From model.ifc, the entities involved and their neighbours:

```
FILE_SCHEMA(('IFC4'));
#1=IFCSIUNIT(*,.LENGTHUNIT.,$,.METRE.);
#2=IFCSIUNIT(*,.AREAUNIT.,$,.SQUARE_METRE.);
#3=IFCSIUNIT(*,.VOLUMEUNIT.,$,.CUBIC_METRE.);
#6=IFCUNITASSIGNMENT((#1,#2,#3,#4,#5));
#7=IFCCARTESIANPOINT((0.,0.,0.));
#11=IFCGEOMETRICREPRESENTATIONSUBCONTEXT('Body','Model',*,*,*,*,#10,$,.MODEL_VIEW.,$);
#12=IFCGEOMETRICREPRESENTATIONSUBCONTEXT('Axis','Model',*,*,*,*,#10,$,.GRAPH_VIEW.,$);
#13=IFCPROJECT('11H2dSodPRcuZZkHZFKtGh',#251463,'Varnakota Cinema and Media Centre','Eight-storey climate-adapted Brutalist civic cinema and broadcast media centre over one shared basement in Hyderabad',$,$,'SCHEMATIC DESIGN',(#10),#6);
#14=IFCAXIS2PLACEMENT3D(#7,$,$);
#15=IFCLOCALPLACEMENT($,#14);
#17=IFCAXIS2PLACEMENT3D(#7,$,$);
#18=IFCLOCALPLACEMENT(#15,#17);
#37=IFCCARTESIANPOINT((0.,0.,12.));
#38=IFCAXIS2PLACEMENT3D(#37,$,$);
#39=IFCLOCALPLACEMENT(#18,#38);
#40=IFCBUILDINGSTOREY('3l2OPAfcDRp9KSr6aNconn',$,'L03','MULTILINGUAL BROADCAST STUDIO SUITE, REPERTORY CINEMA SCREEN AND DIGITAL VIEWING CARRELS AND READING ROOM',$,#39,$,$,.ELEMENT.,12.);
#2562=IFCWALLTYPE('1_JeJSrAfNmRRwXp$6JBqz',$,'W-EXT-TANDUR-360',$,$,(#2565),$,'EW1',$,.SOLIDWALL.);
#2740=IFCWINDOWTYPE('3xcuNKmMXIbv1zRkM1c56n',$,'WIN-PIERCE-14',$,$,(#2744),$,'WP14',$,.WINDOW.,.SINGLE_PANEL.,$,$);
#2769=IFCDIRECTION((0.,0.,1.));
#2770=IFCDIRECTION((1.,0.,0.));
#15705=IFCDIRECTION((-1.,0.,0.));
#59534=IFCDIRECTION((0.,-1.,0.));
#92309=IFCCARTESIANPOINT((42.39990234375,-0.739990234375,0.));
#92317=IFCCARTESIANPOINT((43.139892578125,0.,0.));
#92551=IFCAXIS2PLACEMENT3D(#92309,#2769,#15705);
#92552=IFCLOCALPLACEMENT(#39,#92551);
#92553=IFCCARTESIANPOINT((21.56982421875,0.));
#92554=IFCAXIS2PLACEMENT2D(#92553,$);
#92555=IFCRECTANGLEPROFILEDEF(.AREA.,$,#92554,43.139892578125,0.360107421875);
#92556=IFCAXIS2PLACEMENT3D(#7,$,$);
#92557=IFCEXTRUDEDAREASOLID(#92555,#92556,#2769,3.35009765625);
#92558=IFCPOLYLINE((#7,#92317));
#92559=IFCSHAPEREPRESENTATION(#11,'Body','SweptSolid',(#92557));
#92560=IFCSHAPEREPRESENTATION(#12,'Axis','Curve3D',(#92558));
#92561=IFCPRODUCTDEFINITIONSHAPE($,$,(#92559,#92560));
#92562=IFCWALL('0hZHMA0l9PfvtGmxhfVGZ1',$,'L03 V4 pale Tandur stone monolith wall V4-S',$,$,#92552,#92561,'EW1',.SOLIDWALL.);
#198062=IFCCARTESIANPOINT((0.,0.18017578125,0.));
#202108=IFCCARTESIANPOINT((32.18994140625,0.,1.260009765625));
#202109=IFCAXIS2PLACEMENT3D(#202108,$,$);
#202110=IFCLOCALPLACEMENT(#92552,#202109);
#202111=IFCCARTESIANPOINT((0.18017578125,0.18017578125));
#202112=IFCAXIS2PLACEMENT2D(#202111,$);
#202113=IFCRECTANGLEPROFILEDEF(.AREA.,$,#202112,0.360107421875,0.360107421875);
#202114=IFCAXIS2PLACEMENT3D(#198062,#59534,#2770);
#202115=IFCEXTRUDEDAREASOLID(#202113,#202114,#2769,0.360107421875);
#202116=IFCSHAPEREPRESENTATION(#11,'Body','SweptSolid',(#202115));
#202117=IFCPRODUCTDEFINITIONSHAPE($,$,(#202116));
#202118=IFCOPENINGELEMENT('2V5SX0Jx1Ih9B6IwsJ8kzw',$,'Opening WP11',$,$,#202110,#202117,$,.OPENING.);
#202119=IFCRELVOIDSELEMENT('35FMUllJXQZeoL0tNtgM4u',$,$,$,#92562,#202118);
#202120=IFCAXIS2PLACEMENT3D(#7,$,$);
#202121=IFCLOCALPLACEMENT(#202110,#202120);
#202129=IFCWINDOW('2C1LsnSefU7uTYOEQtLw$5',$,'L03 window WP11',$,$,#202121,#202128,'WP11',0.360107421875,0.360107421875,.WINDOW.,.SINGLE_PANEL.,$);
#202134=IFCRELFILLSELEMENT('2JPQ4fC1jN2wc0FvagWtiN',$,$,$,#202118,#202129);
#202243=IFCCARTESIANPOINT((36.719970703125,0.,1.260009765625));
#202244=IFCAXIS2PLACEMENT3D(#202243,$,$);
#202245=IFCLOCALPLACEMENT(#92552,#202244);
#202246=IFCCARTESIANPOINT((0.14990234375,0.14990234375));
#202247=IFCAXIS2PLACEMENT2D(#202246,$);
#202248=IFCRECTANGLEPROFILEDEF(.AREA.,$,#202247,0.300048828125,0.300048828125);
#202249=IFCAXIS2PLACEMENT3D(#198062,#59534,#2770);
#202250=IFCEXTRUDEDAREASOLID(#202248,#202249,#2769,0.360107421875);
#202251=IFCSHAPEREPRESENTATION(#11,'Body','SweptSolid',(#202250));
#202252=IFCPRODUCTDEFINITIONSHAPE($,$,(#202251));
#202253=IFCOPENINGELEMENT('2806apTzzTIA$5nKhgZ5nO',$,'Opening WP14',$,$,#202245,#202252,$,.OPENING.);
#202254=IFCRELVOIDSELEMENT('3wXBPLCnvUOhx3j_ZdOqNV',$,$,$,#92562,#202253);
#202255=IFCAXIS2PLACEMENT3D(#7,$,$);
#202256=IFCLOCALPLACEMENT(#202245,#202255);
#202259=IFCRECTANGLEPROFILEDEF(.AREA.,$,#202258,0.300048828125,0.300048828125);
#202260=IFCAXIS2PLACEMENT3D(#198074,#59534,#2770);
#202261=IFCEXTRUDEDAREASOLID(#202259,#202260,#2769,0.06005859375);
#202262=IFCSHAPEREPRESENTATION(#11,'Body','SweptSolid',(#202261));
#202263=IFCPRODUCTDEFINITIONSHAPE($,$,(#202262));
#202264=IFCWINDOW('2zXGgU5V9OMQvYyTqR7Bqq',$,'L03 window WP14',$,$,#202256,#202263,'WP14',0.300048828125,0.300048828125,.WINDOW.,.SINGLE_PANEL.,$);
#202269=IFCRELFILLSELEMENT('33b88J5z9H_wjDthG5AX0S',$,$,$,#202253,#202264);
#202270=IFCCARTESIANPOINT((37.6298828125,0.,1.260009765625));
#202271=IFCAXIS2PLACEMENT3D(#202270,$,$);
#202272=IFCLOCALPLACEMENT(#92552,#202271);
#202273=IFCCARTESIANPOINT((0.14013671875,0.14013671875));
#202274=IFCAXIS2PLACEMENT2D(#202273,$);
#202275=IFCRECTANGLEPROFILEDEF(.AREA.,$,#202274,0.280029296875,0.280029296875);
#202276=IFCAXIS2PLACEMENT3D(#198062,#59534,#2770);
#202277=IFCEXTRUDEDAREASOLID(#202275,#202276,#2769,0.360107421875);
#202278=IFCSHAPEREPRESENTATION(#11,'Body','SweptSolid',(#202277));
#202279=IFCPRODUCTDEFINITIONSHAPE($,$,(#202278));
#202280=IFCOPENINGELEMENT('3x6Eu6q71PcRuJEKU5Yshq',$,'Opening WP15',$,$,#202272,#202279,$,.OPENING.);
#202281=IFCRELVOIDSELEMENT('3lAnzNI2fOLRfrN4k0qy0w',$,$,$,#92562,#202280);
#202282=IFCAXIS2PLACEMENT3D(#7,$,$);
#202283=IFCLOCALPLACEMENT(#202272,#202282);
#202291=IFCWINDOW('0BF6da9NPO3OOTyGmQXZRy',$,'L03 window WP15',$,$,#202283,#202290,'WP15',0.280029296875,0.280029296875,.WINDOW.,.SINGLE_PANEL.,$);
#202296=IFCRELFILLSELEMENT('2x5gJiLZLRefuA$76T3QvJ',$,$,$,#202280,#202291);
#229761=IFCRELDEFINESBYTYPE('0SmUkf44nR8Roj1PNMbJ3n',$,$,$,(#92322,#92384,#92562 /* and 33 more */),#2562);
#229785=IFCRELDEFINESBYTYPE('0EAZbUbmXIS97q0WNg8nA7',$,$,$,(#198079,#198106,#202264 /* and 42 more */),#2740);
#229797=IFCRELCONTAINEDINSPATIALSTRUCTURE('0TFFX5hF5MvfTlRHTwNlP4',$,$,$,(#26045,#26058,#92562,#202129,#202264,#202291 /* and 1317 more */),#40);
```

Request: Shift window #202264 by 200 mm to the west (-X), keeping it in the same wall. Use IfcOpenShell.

```python
import ifcopenshell
import ifcopenshell.api.geometry
import ifcopenshell.util.placement
import ifcopenshell.util.unit

model = ifcopenshell.open("model.ifc")
unit_scale = ifcopenshell.util.unit.calculate_unit_scale(model)

window = model.by_guid("2zXGgU5V9OMQvYyTqR7Bqq")
opening = window.FillsVoids[0].RelatingOpeningElement
wall = opening.VoidsElements[0].RelatingBuildingElement

wall_matrix = ifcopenshell.util.placement.get_local_placement(wall.ObjectPlacement)
shift = wall_matrix[:3, 0] * 0.2 / unit_scale
before = ifcopenshell.util.placement.get_local_placement(window.ObjectPlacement)[:3, 3].copy()

# The window is placed relative to its opening, so it follows when the opening moves.
matrix = ifcopenshell.util.placement.get_local_placement(opening.ObjectPlacement)
matrix[:3, 3] += shift
ifcopenshell.api.geometry.edit_object_placement(
    model, product=opening, matrix=matrix, is_si=False, should_transform_children=True
)

after = ifcopenshell.util.placement.get_local_placement(window.ObjectPlacement)[:3, 3]
print("window moved by", (after - before).round(3) + 0.0)

model.write("model_v2.ifc")
```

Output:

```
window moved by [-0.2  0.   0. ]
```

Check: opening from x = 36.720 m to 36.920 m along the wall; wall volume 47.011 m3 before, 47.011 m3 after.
